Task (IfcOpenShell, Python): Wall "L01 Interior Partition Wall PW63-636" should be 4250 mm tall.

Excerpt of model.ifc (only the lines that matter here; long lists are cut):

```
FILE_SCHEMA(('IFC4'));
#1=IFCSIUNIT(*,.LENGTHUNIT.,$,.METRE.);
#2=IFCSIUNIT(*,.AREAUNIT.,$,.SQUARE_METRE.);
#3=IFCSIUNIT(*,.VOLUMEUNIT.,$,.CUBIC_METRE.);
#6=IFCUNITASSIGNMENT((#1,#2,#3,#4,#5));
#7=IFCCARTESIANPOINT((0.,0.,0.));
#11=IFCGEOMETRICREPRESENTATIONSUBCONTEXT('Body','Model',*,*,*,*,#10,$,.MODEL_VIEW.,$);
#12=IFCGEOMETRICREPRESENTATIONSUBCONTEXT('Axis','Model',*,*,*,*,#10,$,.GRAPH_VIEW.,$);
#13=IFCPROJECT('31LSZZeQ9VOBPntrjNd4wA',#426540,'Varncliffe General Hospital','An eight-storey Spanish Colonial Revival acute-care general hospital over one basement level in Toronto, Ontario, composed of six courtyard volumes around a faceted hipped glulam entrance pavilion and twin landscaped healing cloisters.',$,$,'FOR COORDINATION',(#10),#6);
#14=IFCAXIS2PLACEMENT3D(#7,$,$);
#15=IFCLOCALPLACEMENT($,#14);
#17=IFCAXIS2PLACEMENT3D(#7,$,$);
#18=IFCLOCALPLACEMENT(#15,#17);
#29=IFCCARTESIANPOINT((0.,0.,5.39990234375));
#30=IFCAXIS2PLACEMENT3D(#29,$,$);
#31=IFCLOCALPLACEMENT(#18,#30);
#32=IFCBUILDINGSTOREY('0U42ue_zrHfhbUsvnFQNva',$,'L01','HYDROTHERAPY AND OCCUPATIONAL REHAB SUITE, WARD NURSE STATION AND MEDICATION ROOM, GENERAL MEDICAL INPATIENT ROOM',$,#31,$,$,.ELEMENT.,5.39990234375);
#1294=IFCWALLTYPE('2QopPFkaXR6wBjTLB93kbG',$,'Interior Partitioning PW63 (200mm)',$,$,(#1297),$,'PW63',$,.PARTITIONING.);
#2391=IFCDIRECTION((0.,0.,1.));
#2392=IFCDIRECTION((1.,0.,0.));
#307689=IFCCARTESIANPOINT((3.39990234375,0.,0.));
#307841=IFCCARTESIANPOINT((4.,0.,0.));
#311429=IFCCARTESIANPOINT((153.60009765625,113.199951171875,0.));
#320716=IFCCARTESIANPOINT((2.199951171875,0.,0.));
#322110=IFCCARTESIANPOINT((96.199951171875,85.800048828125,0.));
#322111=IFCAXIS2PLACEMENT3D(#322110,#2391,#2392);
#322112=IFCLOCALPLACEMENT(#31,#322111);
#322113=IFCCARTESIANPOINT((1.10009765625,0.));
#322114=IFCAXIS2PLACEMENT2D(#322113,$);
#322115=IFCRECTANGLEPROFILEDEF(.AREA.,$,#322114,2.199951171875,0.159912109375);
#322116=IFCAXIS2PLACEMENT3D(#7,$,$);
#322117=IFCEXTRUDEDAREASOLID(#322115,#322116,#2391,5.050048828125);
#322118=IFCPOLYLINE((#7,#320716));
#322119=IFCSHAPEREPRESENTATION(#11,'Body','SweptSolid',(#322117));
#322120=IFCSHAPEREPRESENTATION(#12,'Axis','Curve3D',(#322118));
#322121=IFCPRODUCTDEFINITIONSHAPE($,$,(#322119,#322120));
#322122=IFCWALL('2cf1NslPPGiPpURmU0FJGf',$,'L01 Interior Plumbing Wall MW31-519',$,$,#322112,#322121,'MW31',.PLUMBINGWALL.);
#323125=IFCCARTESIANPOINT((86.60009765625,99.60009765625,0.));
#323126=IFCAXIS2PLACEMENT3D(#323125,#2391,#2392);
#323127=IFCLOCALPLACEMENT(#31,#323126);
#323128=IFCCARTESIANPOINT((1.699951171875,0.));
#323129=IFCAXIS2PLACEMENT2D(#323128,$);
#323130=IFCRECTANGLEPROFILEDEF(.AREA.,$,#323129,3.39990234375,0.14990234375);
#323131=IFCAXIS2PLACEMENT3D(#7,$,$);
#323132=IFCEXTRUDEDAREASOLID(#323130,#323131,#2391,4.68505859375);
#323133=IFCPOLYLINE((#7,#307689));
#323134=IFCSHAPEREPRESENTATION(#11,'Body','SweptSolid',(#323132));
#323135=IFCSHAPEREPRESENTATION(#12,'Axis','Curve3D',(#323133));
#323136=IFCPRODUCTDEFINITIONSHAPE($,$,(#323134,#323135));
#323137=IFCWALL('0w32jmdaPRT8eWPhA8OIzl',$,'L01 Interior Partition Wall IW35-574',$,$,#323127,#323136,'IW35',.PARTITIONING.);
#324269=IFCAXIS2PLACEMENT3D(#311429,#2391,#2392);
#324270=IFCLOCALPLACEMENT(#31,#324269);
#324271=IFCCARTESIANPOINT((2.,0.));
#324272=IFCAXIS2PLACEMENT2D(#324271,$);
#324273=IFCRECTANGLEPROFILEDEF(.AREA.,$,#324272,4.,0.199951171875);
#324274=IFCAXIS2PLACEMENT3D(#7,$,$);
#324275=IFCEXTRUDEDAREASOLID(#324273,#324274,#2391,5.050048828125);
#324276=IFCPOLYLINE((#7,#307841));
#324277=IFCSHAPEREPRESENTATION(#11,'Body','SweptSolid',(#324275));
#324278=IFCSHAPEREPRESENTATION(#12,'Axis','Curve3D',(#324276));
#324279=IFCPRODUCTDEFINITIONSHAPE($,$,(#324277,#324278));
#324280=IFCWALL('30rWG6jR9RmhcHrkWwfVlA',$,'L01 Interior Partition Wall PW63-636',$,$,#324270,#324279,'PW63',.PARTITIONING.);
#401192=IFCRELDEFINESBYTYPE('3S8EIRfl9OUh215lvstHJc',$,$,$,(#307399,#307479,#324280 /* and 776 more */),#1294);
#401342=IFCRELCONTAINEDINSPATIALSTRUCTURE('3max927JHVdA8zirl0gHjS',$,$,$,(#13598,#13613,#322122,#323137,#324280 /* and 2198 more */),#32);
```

```python
import ifcopenshell
import ifcopenshell.geom
import ifcopenshell.util.representation
import ifcopenshell.util.shape

model = ifcopenshell.open("model.ifc")
settings = ifcopenshell.geom.settings()


def volume(element):
    """Net volume in cubic metres, openings subtracted."""
    shape = ifcopenshell.geom.create_shape(settings, element)
    return ifcopenshell.util.shape.get_volume(shape.geometry)


wall = model.by_guid("30rWG6jR9RmhcHrkWwfVlA")
before = volume(wall)

body = ifcopenshell.util.representation.get_representation(wall, "Model", "Body")
solid = body.Items[0]
old_height = solid.Depth
solid.Depth = 4.25
after = volume(wall)

print(f"height {old_height:g} -> {solid.Depth:g}, volume {before:.3f} -> {after:.3f} m3")

model.write("model_edited.ifc")
```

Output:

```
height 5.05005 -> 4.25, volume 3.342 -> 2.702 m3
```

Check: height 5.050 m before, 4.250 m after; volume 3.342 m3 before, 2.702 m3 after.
